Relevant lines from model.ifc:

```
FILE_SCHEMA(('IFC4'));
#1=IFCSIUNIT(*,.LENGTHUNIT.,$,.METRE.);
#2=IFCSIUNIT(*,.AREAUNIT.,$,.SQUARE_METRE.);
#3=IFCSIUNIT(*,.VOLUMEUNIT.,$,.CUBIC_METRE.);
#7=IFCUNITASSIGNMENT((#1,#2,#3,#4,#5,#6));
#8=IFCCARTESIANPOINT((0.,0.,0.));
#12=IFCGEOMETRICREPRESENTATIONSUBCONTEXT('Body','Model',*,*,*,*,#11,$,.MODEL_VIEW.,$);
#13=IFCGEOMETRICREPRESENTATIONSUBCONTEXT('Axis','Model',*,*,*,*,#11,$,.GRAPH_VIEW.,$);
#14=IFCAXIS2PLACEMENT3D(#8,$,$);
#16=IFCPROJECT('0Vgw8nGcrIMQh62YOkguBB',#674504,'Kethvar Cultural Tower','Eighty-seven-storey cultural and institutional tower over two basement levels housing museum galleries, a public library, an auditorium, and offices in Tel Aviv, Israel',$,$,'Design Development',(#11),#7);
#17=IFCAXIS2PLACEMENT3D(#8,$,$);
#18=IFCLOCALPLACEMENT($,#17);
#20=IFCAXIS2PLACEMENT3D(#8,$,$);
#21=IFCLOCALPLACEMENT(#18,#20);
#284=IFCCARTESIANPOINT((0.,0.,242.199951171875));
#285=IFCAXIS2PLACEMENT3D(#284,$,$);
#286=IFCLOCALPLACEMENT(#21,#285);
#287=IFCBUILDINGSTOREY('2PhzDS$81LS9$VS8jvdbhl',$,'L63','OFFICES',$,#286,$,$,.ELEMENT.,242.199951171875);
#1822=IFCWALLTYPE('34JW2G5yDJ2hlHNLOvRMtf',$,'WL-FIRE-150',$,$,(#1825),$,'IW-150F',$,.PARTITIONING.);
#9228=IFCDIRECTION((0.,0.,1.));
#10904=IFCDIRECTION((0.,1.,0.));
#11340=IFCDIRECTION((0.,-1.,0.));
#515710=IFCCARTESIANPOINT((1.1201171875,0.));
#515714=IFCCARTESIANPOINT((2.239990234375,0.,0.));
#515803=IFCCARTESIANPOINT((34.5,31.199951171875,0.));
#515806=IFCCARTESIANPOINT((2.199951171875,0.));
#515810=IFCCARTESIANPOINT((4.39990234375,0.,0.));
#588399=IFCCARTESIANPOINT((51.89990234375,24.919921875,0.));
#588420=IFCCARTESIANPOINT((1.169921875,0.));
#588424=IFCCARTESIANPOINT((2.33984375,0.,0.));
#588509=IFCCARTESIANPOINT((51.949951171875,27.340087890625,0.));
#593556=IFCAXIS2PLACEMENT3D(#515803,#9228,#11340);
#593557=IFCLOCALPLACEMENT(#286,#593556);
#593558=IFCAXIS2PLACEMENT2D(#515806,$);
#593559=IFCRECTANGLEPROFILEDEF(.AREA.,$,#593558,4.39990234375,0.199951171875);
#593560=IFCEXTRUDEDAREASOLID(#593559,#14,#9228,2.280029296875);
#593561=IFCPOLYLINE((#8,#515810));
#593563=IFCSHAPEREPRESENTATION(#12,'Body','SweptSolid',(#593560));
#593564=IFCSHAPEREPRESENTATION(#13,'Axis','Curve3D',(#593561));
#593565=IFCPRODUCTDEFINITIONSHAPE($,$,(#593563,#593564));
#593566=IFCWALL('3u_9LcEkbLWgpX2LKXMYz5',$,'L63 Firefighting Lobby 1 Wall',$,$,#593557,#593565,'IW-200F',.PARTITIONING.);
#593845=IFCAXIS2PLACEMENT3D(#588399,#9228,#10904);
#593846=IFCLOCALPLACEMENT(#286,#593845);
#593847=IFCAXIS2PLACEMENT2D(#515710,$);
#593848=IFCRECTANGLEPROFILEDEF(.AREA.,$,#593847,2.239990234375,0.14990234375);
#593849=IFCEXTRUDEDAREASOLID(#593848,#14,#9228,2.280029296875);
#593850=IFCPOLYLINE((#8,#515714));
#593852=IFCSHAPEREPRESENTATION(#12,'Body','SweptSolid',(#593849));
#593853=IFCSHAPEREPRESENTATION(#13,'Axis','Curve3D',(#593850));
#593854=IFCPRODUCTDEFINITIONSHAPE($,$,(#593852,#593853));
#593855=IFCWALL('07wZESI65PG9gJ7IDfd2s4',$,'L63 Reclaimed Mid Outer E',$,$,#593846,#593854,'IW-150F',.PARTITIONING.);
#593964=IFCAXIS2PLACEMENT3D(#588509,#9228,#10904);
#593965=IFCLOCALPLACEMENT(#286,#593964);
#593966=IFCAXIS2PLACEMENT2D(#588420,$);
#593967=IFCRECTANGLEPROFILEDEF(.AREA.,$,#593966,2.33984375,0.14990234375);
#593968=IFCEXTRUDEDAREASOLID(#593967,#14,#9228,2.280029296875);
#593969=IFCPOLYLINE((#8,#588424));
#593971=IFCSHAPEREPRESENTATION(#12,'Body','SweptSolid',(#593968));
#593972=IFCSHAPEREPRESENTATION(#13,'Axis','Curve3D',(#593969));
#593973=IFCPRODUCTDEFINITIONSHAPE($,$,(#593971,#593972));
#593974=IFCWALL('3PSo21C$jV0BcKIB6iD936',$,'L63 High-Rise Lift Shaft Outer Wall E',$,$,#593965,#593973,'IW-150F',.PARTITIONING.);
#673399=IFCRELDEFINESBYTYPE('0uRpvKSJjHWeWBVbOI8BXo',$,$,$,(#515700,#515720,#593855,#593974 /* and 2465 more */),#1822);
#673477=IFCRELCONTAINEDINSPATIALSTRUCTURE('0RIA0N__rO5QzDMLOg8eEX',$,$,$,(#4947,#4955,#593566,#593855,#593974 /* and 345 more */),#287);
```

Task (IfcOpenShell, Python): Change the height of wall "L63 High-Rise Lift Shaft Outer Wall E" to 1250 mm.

```python
import ifcopenshell
import ifcopenshell.geom
import ifcopenshell.util.representation
import ifcopenshell.util.shape

model = ifcopenshell.open("model.ifc")
settings = ifcopenshell.geom.settings()


def volume(element):
    """Net volume in cubic metres, openings subtracted."""
    shape = ifcopenshell.geom.create_shape(settings, element)
    return ifcopenshell.util.shape.get_volume(shape.geometry)


wall = model.by_guid("3PSo21C$jV0BcKIB6iD936")
before = volume(wall)

body = ifcopenshell.util.representation.get_representation(wall, "Model", "Body")
solid = body.Items[0]
old_height = solid.Depth
solid.Depth = 1.25
after = volume(wall)

print(f"height {old_height:g} -> {solid.Depth:g}, volume {before:.3f} -> {after:.3f} m3")

model.write("model_updated.ifc")
```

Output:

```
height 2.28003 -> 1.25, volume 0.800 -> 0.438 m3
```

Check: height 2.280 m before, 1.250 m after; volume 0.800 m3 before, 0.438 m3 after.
